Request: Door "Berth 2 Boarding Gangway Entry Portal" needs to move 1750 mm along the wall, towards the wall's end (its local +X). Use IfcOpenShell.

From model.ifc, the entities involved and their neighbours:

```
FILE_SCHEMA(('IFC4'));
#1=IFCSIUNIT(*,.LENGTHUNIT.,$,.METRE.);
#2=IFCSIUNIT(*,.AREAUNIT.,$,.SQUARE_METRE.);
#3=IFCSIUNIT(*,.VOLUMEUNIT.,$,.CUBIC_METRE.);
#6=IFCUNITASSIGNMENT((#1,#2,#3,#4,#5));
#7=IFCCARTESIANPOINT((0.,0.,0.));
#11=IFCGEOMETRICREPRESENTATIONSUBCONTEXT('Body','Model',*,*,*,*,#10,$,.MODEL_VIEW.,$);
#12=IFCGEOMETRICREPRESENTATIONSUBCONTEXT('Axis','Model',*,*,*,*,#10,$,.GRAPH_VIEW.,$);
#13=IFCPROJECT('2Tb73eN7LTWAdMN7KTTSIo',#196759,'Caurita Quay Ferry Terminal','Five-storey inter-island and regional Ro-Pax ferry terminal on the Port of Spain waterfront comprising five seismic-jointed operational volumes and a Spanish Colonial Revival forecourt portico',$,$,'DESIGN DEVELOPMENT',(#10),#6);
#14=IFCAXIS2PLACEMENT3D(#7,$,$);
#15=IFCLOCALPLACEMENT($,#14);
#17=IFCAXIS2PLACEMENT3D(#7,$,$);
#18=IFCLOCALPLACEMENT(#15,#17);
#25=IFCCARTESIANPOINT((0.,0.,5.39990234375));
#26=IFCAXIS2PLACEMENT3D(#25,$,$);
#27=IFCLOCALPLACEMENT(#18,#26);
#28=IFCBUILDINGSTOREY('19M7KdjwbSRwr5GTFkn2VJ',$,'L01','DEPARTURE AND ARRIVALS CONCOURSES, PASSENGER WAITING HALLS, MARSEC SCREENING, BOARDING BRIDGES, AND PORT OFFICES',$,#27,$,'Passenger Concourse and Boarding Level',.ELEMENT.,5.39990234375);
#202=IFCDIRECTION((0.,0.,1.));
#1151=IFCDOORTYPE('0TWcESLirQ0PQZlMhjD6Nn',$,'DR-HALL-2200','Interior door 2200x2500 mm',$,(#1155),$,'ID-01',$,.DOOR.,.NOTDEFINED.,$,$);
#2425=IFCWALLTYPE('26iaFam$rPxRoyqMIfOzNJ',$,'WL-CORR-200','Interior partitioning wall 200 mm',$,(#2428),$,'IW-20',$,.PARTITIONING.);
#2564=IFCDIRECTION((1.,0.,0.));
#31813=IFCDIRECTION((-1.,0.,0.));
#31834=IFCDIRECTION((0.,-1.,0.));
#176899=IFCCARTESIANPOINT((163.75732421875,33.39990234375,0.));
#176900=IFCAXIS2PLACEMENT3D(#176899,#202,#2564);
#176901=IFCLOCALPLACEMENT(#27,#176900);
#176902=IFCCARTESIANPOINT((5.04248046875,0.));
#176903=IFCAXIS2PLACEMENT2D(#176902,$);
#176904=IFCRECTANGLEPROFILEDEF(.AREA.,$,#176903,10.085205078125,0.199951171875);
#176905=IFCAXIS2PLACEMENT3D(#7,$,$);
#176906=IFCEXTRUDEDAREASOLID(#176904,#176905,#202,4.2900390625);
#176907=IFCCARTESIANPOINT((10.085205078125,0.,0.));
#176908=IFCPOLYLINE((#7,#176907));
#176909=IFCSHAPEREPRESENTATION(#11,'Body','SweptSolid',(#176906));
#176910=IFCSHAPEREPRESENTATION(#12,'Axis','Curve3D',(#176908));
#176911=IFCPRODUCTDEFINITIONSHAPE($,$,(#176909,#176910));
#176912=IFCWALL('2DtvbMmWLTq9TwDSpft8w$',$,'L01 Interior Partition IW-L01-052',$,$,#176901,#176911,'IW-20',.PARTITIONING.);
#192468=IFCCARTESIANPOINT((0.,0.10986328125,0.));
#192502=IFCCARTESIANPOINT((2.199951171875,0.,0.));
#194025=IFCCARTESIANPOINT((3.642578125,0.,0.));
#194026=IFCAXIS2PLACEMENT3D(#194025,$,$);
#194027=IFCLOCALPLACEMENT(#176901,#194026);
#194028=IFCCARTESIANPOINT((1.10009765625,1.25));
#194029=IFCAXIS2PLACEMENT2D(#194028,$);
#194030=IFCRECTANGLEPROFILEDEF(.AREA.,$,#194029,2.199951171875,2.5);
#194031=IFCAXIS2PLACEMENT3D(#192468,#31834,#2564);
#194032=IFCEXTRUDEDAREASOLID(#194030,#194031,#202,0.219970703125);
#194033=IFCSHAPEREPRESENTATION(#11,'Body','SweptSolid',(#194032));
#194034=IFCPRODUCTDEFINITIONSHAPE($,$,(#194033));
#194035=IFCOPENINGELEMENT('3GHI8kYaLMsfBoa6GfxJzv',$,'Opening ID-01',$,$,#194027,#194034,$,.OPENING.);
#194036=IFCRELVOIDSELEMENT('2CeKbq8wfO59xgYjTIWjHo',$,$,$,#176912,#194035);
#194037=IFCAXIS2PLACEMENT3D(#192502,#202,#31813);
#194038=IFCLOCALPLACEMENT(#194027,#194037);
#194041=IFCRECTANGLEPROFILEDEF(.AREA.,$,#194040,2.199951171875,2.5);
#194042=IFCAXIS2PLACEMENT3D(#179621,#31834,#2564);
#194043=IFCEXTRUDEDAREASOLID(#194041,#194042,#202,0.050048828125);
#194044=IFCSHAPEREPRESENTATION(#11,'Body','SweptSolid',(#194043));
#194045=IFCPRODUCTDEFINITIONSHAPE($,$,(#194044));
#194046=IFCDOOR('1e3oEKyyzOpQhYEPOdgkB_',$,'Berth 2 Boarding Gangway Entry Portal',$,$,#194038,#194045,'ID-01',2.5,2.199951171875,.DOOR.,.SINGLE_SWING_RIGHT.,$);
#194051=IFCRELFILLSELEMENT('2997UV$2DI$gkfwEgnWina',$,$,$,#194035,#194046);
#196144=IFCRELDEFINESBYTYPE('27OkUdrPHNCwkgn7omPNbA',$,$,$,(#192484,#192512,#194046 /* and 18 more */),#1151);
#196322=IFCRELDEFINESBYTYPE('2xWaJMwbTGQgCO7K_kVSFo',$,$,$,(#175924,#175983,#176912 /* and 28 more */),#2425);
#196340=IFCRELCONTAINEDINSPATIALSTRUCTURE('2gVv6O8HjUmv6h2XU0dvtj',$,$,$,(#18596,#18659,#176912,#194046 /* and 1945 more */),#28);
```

```python
import ifcopenshell
import ifcopenshell.api.geometry
import ifcopenshell.util.placement

model = ifcopenshell.open("model.ifc")

door = model.by_guid("1e3oEKyyzOpQhYEPOdgkB_")
opening = door.FillsVoids[0].RelatingOpeningElement
wall = opening.VoidsElements[0].RelatingBuildingElement

wall_matrix = ifcopenshell.util.placement.get_local_placement(wall.ObjectPlacement)
shift = wall_matrix[:3, 0] * 1.75
before = ifcopenshell.util.placement.get_local_placement(door.ObjectPlacement)[:3, 3].copy()

# The door is placed relative to its opening, so it follows when the opening moves.
matrix = ifcopenshell.util.placement.get_local_placement(opening.ObjectPlacement)
matrix[:3, 3] += shift
ifcopenshell.api.geometry.edit_object_placement(
    model, product=opening, matrix=matrix, is_si=False, should_transform_children=True
)

after = ifcopenshell.util.placement.get_local_placement(door.ObjectPlacement)[:3, 3]
print("door moved by", (after - before).round(3) + 0.0)

model.write("model-out.ifc")
```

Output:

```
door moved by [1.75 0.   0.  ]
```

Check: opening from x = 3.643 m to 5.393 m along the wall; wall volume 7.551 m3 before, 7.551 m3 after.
